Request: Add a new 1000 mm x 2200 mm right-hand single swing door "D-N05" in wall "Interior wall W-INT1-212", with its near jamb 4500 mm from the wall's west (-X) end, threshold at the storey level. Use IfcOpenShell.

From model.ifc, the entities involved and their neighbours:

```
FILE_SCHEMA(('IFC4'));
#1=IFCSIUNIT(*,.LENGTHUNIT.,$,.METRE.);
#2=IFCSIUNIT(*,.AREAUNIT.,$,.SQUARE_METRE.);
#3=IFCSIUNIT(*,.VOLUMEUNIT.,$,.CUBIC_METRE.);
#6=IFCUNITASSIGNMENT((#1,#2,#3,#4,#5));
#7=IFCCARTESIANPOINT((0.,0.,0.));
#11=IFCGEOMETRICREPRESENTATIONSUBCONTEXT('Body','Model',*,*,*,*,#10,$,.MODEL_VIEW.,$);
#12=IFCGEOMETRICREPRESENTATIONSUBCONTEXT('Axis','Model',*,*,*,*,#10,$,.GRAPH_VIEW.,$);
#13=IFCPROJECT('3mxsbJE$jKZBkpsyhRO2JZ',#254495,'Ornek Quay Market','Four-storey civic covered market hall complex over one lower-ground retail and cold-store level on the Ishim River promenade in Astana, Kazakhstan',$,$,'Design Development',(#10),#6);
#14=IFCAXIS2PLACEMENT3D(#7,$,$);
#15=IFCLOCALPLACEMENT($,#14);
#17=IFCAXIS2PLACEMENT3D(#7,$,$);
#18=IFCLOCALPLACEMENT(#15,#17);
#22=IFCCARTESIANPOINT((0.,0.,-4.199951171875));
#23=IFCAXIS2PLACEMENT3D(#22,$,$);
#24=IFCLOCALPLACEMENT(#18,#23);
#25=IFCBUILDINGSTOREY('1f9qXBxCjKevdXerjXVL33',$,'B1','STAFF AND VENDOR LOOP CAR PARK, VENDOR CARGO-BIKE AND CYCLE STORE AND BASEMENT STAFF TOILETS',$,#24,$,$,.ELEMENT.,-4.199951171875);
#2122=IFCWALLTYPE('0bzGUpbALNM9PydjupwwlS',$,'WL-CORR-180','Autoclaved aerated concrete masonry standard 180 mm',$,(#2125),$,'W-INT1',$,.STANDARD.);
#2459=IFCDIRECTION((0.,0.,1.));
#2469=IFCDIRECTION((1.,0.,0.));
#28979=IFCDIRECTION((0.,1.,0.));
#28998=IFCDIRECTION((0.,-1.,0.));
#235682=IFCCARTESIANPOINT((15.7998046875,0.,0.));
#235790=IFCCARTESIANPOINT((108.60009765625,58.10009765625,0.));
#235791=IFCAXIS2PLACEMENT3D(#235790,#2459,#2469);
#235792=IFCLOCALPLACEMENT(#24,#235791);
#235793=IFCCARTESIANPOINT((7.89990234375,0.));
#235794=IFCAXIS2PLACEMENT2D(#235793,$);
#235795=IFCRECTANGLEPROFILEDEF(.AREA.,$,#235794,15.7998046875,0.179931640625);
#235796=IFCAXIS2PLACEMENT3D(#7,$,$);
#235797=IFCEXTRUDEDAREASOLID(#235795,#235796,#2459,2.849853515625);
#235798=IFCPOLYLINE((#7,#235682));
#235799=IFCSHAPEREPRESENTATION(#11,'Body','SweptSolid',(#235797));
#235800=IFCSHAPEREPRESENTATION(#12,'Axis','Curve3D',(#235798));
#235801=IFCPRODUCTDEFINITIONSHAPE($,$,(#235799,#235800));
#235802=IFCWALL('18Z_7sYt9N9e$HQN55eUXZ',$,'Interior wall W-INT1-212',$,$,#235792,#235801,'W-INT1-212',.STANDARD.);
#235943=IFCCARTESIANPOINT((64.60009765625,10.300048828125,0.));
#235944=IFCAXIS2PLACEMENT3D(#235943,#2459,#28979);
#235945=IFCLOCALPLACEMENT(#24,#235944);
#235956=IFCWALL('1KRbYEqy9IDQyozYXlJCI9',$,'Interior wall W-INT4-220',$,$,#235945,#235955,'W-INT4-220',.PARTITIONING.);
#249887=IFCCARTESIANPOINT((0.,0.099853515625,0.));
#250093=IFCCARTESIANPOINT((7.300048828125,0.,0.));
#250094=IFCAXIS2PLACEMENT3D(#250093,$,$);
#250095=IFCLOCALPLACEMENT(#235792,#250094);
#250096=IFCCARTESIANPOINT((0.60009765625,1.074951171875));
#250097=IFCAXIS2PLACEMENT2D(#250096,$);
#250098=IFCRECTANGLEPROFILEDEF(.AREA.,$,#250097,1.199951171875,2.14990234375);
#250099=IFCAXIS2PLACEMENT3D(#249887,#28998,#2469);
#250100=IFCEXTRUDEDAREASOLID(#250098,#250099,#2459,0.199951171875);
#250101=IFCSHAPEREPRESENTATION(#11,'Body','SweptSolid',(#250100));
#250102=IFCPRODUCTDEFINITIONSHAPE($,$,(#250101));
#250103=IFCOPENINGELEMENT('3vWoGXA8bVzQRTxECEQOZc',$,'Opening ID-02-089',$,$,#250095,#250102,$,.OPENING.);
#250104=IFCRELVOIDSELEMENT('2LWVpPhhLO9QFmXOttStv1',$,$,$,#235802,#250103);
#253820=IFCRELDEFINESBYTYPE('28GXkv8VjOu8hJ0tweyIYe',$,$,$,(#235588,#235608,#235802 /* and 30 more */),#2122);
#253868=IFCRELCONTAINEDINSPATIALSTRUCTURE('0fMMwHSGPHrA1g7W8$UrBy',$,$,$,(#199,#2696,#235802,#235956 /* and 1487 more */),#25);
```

```python
import numpy as np
import ifcopenshell
import ifcopenshell.api.feature
import ifcopenshell.api.geometry
import ifcopenshell.api.root
import ifcopenshell.api.spatial
import ifcopenshell.geom
import ifcopenshell.util.element
import ifcopenshell.util.placement
import ifcopenshell.util.representation
import ifcopenshell.util.shape
import ifcopenshell.util.unit

model = ifcopenshell.open("model.ifc")
unit_scale = ifcopenshell.util.unit.calculate_unit_scale(model)
settings = ifcopenshell.geom.settings()


def volume(element):
    """Net volume in cubic metres, openings subtracted."""
    shape = ifcopenshell.geom.create_shape(settings, element)
    return ifcopenshell.util.shape.get_volume(shape.geometry)


wall = model.by_guid("18Z_7sYt9N9e$HQN55eUXZ")
storey = ifcopenshell.util.element.get_container(wall, ifc_class="IfcBuildingStorey")
context = ifcopenshell.util.representation.get_context(model, "Model", "Body", "MODEL_VIEW")
before = volume(wall)

width, height, from_end, sill = 1, 2.2, 4.5, 0.0  # metres

# The wall runs along its own X axis, and the end named is its -X end.
wall_shape = ifcopenshell.geom.create_shape(settings, wall)
x, y, z = ifcopenshell.util.shape.get_vertices(wall_shape.geometry).T
start = x.min() + from_end
face, thickness = float(y.min()), float(y.max() - y.min())
wall_matrix = ifcopenshell.util.placement.get_local_placement(wall.ObjectPlacement)
level = ifcopenshell.util.placement.get_local_placement(storey.ObjectPlacement)[2, 3]


def in_wall(x, y):
    """Placement at x, y metres in the wall's axes, at sill height."""
    matrix = wall_matrix.copy()
    matrix[:, 3] = wall_matrix @ np.array([x / unit_scale, y / unit_scale, 0.0, 1.0])
    matrix[2, 3] = level + sill / unit_scale
    return matrix


# Opening: a box that overshoots both wall faces by 50 mm.
opening = ifcopenshell.api.root.create_entity(model, ifc_class="IfcOpeningElement", predefined_type="OPENING")
box = ifcopenshell.api.geometry.add_wall_representation(
    model, context=context, length=width, height=height, thickness=thickness + 0.1
)
ifcopenshell.api.geometry.assign_representation(model, product=opening, representation=box)
ifcopenshell.api.geometry.edit_object_placement(model, product=opening, matrix=in_wall(start, face - 0.05), is_si=False)
ifcopenshell.api.feature.add_feature(model, feature=opening, element=wall)

door = ifcopenshell.api.root.create_entity(model, ifc_class="IfcDoor", name="D-N05", predefined_type="DOOR")
door.OverallWidth, door.OverallHeight = width / unit_scale, height / unit_scale
door.OperationType = "SINGLE_SWING_RIGHT"
body = ifcopenshell.api.geometry.add_door_representation(
    model,
    context=context,
    overall_width=door.OverallWidth,
    overall_height=door.OverallHeight,
    operation_type="SINGLE_SWING_RIGHT",
    lining_properties={"LiningDepth": thickness / unit_scale, "ThresholdDepth": thickness / unit_scale},
)
ifcopenshell.api.geometry.assign_representation(model, product=door, representation=body)
ifcopenshell.api.spatial.assign_container(model, products=[door], relating_structure=storey)
ifcopenshell.api.feature.add_filling(model, opening=opening, element=door)

# The lining spans the wall, so the door starts at the wall face.
ifcopenshell.api.geometry.edit_object_placement(model, product=door, matrix=in_wall(start, face), is_si=False)

after = volume(wall)

print(f"wall volume {before:.3f} -> {after:.3f} m3")

model.write("model-out.ifc")
```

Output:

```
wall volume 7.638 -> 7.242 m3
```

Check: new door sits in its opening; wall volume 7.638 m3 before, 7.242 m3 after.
